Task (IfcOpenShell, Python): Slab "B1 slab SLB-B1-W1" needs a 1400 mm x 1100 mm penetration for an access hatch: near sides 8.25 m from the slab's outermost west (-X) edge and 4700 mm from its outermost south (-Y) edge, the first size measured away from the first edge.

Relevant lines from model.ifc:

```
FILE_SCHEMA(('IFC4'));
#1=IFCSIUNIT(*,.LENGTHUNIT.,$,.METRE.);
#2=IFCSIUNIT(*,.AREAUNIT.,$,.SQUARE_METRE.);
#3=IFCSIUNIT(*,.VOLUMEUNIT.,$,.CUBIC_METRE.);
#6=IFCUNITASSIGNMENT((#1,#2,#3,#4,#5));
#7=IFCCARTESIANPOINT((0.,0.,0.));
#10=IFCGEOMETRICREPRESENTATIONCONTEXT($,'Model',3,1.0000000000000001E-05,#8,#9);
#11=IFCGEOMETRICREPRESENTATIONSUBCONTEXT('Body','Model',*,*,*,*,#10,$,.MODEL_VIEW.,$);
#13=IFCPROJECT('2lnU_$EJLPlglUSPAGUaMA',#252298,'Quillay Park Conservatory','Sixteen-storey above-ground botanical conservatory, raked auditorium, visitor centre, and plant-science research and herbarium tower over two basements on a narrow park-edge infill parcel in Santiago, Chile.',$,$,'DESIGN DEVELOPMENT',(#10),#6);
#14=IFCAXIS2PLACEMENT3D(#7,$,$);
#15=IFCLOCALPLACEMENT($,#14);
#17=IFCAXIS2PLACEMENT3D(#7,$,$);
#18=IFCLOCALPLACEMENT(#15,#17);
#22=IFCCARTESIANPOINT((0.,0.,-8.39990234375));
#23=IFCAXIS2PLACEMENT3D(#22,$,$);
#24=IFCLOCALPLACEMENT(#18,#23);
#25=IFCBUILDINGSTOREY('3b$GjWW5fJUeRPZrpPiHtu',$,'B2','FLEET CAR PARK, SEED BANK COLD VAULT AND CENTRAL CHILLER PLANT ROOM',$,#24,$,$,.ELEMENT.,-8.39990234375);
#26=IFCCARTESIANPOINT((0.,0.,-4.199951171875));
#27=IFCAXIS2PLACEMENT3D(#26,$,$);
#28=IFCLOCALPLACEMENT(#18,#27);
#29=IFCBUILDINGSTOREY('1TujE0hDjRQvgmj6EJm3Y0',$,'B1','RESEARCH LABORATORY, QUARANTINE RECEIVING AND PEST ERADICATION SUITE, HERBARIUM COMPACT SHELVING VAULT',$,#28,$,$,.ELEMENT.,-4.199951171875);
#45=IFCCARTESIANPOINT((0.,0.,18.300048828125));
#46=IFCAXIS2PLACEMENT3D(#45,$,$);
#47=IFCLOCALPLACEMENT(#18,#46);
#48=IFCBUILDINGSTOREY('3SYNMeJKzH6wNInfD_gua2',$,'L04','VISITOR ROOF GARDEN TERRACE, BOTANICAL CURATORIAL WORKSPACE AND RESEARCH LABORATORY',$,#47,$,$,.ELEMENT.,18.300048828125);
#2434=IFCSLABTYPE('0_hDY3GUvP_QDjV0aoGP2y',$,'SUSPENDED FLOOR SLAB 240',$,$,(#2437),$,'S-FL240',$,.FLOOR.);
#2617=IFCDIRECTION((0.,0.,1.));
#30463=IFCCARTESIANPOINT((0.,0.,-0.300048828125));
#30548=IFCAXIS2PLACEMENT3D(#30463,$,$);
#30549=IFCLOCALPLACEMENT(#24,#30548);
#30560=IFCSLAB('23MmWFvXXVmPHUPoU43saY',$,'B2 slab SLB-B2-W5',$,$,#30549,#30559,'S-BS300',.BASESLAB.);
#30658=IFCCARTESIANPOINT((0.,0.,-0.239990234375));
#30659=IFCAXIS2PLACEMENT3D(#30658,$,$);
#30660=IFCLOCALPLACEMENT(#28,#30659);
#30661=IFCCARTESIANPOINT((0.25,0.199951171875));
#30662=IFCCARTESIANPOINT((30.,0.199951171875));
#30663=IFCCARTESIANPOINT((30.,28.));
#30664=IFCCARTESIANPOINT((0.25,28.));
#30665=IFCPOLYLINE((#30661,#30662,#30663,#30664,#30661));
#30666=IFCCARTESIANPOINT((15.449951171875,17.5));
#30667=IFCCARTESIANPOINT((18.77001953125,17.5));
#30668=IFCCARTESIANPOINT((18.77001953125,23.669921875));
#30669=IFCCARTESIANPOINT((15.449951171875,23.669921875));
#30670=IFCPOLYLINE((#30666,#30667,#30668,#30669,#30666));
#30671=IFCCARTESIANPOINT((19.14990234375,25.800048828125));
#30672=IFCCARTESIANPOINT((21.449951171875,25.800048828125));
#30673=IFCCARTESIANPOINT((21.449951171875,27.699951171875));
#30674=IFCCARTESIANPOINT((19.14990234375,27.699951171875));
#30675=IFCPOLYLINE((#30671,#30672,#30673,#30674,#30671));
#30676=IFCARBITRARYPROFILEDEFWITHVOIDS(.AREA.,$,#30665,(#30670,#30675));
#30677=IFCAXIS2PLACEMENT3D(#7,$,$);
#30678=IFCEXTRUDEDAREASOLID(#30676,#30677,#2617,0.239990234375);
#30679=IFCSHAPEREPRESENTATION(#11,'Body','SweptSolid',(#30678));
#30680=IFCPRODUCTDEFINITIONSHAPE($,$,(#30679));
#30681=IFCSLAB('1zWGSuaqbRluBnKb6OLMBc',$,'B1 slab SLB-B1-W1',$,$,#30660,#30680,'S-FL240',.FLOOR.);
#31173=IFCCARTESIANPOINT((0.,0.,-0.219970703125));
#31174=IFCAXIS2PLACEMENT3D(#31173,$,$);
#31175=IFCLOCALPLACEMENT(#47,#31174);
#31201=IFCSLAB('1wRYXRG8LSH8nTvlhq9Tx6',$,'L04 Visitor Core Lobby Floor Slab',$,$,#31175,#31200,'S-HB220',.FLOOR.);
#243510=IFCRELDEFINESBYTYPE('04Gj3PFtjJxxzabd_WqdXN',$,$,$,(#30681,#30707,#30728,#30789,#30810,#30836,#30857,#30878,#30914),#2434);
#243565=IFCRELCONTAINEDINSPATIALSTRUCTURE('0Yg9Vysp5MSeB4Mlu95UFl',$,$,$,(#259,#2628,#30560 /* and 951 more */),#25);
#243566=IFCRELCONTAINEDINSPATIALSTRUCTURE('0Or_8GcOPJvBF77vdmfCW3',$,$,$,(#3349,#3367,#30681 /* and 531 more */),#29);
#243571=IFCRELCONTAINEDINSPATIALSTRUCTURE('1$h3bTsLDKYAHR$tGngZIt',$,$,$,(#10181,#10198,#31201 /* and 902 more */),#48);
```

```python
import numpy as np
import ifcopenshell
import ifcopenshell.api.feature
import ifcopenshell.api.geometry
import ifcopenshell.api.root
import ifcopenshell.geom
import ifcopenshell.util.placement
import ifcopenshell.util.representation
import ifcopenshell.util.shape
import ifcopenshell.util.unit

model = ifcopenshell.open("model.ifc")
unit_scale = ifcopenshell.util.unit.calculate_unit_scale(model)
settings = ifcopenshell.geom.settings()


def volume(element):
    """Net volume in cubic metres, openings subtracted."""
    shape = ifcopenshell.geom.create_shape(settings, element)
    return ifcopenshell.util.shape.get_volume(shape.geometry)


slab = model.by_guid("1zWGSuaqbRluBnKb6OLMBc")
before = volume(slab)

# Extent in the slab's own axes, in metres. The edges named are its -X and -Y sides.
slab_shape = ifcopenshell.geom.create_shape(settings, slab)
vertices = ifcopenshell.util.shape.get_vertices(slab_shape.geometry)
x_min, y_min, bottom = vertices.min(axis=0)
top = vertices[:, 2].max()

opening = ifcopenshell.api.root.create_entity(model, ifc_class="IfcOpeningElement", name="Access hatch opening", predefined_type="OPENING")
context = ifcopenshell.util.representation.get_context(model, "Model", "Body", "MODEL_VIEW")
width, depth = 1.4, 1.1
outline = [(0.0, 0.0), (width, 0.0), (width, depth), (0.0, depth), (0.0, 0.0)]
# Overshoot both faces by 50 mm so the cut is clean.
shape = ifcopenshell.api.geometry.add_slab_representation(
    model, context=context, depth=top - bottom + 0.1, polyline=outline
)
ifcopenshell.api.geometry.assign_representation(model, product=opening, representation=shape)

matrix = ifcopenshell.util.placement.get_local_placement(slab.ObjectPlacement)
matrix[:, 3] = matrix @ np.append(np.array([x_min + 8.25, y_min + 4.7, bottom - 0.05]) / unit_scale, 1.0)
ifcopenshell.api.geometry.edit_object_placement(model, product=opening, matrix=matrix, is_si=False)
ifcopenshell.api.feature.add_feature(model, feature=opening, element=slab)

after = volume(slab)

print(f"slab volume {before:.3f} -> {after:.3f} m3")

model.write("model_rev.ifc")
```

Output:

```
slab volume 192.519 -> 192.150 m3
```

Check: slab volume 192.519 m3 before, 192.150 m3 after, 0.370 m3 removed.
